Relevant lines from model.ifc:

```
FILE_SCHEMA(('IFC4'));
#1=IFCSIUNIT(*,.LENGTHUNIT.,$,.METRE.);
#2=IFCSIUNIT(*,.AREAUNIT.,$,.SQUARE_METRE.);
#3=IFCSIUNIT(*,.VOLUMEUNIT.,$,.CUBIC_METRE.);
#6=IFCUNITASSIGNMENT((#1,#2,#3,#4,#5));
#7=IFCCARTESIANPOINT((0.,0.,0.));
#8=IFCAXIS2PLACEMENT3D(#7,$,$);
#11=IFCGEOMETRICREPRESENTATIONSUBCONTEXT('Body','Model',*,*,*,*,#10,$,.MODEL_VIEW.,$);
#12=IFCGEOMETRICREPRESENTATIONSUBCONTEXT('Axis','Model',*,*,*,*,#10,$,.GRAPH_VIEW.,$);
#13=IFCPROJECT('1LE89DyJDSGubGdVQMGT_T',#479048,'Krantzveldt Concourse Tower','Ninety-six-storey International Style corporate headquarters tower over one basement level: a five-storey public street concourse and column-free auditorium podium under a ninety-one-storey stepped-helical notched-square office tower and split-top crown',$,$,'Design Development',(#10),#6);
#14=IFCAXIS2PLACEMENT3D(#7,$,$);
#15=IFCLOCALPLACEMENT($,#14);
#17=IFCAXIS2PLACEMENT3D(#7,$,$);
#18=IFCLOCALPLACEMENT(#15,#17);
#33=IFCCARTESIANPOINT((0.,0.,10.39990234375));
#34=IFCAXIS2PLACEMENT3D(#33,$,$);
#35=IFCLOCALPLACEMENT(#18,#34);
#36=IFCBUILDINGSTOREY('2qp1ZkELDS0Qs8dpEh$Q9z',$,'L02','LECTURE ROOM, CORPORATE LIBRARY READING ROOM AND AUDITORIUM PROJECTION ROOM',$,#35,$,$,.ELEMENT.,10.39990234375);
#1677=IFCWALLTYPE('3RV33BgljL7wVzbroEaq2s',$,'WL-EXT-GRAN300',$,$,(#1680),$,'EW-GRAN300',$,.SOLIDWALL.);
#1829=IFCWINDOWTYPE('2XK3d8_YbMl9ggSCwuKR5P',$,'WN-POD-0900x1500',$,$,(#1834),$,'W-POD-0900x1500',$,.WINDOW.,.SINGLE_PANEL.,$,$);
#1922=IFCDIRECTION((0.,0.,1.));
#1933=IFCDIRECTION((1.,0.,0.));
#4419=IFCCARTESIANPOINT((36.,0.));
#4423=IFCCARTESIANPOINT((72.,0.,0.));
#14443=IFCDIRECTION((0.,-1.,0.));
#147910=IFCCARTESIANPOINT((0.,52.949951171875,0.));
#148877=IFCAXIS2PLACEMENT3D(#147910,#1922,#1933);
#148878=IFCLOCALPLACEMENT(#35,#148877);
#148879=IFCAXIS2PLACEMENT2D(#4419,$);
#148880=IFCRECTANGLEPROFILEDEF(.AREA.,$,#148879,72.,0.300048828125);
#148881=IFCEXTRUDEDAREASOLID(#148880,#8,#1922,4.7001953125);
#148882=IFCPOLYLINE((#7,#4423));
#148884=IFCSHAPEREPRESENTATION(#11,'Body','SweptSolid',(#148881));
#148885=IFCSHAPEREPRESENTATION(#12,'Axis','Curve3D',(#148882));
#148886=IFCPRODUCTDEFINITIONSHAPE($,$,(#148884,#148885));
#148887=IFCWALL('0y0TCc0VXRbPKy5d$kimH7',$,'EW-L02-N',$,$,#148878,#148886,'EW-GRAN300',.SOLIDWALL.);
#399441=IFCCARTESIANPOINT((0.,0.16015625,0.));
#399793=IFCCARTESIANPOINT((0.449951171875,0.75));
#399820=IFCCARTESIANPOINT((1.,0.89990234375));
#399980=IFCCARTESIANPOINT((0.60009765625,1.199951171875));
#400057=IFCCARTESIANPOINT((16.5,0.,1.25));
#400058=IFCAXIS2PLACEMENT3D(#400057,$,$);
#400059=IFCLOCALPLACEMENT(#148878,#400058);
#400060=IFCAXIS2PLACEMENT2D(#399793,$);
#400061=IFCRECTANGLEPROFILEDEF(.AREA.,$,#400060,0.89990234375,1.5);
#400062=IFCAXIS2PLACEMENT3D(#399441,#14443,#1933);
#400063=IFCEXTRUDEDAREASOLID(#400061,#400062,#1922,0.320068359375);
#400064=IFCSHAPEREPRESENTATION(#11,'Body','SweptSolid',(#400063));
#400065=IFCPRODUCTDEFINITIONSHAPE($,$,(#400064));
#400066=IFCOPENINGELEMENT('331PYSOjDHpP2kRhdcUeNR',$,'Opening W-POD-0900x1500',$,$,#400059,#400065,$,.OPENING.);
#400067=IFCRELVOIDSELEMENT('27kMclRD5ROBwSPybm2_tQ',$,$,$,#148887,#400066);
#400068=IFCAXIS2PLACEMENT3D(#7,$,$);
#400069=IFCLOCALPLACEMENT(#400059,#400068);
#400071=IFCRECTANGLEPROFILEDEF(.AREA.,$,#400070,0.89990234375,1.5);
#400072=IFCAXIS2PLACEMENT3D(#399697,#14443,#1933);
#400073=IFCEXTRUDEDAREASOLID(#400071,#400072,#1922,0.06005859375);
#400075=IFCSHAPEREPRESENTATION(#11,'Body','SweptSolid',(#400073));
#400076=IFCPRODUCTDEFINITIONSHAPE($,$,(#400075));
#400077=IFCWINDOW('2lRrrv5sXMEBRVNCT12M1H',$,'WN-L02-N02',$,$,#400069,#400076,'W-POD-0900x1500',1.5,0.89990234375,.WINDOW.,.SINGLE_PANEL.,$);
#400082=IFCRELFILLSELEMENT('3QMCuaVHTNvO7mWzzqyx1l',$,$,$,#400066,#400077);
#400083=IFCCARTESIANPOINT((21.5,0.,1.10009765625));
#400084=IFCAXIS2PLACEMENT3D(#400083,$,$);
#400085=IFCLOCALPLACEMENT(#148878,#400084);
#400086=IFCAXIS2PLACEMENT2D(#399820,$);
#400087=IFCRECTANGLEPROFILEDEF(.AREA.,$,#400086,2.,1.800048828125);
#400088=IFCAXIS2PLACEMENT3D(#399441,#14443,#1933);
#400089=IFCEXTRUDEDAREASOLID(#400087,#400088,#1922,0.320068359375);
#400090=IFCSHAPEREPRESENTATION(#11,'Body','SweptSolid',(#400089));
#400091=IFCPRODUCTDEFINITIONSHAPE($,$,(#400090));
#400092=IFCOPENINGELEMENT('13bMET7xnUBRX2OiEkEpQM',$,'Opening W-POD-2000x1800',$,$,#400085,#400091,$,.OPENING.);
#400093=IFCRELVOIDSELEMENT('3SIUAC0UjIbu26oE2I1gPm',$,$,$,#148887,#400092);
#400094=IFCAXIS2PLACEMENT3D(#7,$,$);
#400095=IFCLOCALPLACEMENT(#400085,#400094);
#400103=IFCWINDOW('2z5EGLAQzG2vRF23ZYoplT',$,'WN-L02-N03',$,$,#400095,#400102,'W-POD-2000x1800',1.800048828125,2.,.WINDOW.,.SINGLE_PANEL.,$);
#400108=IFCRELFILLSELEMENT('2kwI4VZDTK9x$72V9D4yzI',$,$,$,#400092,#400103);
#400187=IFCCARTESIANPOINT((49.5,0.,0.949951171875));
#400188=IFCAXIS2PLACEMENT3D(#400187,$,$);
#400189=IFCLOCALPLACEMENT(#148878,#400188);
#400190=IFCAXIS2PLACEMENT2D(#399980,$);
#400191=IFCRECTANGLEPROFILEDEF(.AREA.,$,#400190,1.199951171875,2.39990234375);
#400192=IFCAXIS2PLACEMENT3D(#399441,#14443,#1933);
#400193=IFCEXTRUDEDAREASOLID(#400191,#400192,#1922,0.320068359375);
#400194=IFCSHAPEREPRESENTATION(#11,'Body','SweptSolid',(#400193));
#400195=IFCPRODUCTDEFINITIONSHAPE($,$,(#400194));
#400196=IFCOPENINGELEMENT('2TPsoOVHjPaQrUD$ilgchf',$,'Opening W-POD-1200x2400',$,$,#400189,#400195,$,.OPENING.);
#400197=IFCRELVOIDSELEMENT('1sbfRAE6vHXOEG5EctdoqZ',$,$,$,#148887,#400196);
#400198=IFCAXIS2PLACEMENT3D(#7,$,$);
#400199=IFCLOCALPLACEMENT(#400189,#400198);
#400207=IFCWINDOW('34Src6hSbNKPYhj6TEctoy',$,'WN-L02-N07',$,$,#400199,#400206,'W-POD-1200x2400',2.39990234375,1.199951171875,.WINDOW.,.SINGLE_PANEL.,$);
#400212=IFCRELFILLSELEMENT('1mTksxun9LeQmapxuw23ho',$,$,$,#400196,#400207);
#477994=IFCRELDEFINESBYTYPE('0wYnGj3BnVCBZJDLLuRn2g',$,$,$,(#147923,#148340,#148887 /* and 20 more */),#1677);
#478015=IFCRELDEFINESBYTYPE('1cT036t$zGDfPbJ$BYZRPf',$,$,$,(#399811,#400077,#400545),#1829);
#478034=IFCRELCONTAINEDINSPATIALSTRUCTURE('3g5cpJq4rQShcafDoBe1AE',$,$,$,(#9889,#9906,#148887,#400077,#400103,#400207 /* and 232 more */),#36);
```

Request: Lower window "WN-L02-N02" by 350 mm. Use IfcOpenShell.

```python
import numpy as np
import ifcopenshell
import ifcopenshell.api.geometry
import ifcopenshell.util.placement
import ifcopenshell.util.unit

model = ifcopenshell.open("model.ifc")
unit_scale = ifcopenshell.util.unit.calculate_unit_scale(model)

window = model.by_guid("2lRrrv5sXMEBRVNCT12M1H")
opening = window.FillsVoids[0].RelatingOpeningElement
dz = -0.35

shift = np.array([0.0, 0.0, dz])
# The window is placed relative to its opening, so it follows when the opening moves.
matrix = ifcopenshell.util.placement.get_local_placement(opening.ObjectPlacement)
matrix[:3, 3] += shift
ifcopenshell.api.geometry.edit_object_placement(
    model, product=opening, matrix=matrix, is_si=False, should_transform_children=True
)

print(f"moved by {dz * unit_scale:+.3f} m")

model.write("model_rev.ifc")
```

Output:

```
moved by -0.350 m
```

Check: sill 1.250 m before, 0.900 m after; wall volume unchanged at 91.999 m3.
